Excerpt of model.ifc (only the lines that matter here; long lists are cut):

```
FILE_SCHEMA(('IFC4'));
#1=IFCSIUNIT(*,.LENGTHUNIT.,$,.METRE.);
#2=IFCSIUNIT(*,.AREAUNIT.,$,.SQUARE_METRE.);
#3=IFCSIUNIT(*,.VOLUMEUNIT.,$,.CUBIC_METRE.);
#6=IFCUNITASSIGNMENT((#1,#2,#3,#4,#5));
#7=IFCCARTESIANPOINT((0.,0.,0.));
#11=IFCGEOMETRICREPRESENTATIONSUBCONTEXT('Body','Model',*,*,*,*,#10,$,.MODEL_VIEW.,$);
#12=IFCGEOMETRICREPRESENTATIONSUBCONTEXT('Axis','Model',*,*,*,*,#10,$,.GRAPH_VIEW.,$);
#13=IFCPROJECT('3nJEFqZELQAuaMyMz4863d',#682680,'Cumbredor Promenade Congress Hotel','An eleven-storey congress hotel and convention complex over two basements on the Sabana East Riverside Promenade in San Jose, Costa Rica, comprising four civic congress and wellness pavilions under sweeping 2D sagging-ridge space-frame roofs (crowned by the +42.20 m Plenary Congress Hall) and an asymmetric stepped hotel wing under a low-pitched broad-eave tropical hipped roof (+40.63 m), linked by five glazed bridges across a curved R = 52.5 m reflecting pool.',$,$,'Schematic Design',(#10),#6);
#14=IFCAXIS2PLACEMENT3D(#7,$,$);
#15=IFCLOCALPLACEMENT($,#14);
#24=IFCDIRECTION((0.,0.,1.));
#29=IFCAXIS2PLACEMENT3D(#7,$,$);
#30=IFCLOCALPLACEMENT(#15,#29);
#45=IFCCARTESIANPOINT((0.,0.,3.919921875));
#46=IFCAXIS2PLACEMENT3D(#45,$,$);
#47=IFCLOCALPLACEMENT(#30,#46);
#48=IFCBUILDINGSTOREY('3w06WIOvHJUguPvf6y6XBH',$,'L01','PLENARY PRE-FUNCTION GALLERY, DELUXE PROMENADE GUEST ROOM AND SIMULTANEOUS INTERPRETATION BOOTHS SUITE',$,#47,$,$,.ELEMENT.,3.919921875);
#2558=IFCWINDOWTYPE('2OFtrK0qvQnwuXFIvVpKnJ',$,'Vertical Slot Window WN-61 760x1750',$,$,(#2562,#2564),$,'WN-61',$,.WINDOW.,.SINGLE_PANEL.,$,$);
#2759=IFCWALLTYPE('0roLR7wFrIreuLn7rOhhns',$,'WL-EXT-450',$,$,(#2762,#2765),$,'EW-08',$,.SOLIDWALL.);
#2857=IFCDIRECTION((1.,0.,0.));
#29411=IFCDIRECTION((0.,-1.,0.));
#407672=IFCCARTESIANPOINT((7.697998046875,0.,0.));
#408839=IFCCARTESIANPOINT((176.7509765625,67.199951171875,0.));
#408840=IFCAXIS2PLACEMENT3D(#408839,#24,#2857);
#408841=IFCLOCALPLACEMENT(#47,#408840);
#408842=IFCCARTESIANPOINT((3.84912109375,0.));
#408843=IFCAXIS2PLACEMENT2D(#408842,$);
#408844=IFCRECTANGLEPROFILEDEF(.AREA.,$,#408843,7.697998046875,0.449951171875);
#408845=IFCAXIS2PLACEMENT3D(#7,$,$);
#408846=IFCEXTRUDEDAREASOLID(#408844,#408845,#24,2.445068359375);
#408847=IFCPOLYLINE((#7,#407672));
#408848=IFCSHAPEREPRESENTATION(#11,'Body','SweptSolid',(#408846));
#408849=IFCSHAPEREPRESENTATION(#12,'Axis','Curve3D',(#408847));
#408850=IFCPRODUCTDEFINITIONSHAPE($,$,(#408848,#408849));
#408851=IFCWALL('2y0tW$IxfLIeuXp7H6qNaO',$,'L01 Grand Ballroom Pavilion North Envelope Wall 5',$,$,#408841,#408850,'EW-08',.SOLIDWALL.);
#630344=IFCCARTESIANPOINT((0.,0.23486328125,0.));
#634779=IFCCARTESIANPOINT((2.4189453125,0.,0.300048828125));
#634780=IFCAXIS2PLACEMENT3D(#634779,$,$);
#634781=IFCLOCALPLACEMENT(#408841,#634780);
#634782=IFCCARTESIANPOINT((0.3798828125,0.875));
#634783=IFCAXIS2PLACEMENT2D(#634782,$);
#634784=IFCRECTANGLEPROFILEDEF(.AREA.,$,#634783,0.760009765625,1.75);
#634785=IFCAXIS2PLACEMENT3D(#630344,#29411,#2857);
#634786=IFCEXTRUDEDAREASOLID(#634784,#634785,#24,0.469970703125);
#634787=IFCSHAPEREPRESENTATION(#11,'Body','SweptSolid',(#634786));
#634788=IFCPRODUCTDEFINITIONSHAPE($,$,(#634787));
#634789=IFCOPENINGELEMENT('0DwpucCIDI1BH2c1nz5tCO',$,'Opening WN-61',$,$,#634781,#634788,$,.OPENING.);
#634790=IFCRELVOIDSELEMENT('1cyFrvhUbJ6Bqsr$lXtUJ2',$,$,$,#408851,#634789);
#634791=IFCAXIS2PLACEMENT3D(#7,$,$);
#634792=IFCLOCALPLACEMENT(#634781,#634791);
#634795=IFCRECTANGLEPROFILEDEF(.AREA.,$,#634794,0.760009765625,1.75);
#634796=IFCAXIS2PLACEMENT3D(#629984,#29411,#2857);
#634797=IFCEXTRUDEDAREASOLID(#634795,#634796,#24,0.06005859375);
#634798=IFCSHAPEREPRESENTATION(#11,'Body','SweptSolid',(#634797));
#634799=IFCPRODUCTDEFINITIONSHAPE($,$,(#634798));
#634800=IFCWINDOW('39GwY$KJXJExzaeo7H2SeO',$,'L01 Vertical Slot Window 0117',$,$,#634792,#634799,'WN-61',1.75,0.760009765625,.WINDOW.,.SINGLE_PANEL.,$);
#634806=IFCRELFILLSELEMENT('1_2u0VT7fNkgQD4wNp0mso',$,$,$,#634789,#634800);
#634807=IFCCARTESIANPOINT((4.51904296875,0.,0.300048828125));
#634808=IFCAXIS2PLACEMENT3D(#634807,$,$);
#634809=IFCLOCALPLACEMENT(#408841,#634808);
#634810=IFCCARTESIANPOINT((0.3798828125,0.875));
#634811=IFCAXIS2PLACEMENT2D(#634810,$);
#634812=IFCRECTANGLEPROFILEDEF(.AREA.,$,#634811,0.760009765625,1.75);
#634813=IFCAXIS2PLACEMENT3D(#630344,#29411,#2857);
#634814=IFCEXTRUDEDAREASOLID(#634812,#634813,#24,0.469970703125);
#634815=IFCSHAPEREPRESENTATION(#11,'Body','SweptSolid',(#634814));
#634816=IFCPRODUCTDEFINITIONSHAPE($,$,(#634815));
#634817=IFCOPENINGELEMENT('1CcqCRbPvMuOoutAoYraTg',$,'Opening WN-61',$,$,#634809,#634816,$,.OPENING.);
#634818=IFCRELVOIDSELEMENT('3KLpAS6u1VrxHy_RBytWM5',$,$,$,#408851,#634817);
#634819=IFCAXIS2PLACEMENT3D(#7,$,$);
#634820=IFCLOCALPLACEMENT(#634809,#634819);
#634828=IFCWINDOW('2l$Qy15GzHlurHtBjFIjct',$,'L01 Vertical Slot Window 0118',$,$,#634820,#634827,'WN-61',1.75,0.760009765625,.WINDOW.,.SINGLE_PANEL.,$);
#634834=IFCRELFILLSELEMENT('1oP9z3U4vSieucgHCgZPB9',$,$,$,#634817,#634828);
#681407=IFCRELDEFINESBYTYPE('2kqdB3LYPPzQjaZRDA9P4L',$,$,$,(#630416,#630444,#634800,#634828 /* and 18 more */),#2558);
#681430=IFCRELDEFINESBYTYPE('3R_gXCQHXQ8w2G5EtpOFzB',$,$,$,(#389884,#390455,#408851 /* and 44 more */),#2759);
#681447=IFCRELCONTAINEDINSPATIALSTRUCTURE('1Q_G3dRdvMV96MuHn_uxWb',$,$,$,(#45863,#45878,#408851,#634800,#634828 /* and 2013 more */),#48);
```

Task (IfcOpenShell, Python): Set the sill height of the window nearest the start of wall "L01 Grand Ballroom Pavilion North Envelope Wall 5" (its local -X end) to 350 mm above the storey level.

```python
import numpy as np
import ifcopenshell
import ifcopenshell.api.geometry
import ifcopenshell.geom
import ifcopenshell.util.element
import ifcopenshell.util.placement
import ifcopenshell.util.shape
import ifcopenshell.util.unit

model = ifcopenshell.open("model.ifc")
unit_scale = ifcopenshell.util.unit.calculate_unit_scale(model)

window = model.by_guid("39GwY$KJXJExzaeo7H2SeO")
opening = window.FillsVoids[0].RelatingOpeningElement
storey = ifcopenshell.util.element.get_container(window, ifc_class="IfcBuildingStorey")
level = ifcopenshell.util.placement.get_local_placement(storey.ObjectPlacement)[2, 3]

# The opening's origin need not be at the sill, so measure its lowest point.
shape = ifcopenshell.geom.create_shape(ifcopenshell.geom.settings(), opening)
bottom = ifcopenshell.util.shape.get_shape_bottom_elevation(shape, shape.geometry) / unit_scale
dz = level + 0.35 - bottom

shift = np.array([0.0, 0.0, dz])
# The window is placed relative to its opening, so it follows when the opening moves.
matrix = ifcopenshell.util.placement.get_local_placement(opening.ObjectPlacement)
matrix[:3, 3] += shift
ifcopenshell.api.geometry.edit_object_placement(
    model, product=opening, matrix=matrix, is_si=False, should_transform_children=True
)

print(f"moved by {dz * unit_scale:+.3f} m")

model.write("model_updated.ifc")
```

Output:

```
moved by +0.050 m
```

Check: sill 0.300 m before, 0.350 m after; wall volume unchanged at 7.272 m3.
